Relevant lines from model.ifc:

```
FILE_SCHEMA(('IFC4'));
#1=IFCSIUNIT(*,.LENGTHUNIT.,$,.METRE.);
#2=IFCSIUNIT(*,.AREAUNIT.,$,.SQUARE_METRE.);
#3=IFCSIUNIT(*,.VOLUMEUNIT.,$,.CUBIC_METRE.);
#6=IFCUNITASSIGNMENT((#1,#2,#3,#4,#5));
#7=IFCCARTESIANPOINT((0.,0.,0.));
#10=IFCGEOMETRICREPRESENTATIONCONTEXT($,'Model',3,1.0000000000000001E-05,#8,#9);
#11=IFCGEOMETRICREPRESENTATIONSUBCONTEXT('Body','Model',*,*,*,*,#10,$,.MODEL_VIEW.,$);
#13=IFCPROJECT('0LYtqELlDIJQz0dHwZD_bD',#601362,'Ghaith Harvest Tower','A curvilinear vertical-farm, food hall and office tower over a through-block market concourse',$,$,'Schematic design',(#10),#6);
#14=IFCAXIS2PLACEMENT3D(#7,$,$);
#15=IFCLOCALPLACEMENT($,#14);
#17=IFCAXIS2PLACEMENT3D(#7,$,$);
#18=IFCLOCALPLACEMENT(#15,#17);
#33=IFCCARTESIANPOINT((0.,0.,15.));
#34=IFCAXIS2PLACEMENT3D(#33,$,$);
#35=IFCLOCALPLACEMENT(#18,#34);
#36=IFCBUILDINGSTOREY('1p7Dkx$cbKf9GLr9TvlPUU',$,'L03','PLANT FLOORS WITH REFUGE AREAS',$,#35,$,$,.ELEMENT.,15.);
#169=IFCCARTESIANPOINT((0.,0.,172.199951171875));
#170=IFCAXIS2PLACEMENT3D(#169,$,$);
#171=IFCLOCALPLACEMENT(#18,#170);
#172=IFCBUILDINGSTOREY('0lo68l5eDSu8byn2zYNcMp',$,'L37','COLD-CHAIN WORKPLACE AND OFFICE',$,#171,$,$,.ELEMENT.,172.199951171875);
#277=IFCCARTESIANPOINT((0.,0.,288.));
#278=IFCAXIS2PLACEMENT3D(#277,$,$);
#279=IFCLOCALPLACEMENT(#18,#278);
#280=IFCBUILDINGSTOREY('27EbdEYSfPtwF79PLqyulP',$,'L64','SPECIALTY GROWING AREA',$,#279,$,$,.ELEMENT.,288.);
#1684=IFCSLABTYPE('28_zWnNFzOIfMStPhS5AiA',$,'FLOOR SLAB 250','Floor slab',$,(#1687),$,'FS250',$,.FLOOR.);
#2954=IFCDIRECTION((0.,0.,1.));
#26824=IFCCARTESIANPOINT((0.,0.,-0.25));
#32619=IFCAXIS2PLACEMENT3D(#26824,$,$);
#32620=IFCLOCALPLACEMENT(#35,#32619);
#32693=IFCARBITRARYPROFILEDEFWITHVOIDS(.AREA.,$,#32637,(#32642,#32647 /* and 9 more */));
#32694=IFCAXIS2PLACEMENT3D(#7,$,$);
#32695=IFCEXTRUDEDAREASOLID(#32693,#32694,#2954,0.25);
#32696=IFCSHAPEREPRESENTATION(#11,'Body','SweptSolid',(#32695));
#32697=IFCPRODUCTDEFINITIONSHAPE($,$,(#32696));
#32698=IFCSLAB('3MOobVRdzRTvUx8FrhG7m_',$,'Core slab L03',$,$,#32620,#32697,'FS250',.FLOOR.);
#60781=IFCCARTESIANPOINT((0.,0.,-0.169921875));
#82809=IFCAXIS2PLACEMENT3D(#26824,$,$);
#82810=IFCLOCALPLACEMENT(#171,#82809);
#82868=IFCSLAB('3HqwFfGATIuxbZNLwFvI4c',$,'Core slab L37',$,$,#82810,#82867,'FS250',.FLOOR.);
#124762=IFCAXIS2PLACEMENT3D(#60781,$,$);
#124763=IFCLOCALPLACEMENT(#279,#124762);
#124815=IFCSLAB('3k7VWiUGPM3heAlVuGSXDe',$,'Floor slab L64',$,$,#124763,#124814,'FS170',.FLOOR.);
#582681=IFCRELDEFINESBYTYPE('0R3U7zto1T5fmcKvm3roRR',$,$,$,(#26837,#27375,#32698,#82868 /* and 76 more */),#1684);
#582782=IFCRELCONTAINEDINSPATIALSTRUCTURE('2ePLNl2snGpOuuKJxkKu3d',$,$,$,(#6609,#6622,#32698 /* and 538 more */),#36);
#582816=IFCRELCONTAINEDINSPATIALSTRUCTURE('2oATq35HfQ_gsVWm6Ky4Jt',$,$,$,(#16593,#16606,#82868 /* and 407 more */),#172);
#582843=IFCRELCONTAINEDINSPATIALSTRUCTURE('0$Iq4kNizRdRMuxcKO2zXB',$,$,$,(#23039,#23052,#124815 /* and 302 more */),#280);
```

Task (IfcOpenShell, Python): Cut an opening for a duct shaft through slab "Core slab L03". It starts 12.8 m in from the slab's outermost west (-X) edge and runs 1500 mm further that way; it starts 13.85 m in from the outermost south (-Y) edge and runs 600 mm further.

```python
import numpy as np
import ifcopenshell
import ifcopenshell.api.feature
import ifcopenshell.api.geometry
import ifcopenshell.api.root
import ifcopenshell.geom
import ifcopenshell.util.placement
import ifcopenshell.util.representation
import ifcopenshell.util.shape
import ifcopenshell.util.unit

model = ifcopenshell.open("model.ifc")
unit_scale = ifcopenshell.util.unit.calculate_unit_scale(model)
settings = ifcopenshell.geom.settings()


def volume(element):
    """Net volume in cubic metres, openings subtracted."""
    shape = ifcopenshell.geom.create_shape(settings, element)
    return ifcopenshell.util.shape.get_volume(shape.geometry)


slab = model.by_guid("3MOobVRdzRTvUx8FrhG7m_")
before = volume(slab)

# Extent in the slab's own axes, in metres. The edges named are its -X and -Y sides.
slab_shape = ifcopenshell.geom.create_shape(settings, slab)
vertices = ifcopenshell.util.shape.get_vertices(slab_shape.geometry)
x_min, y_min, bottom = vertices.min(axis=0)
top = vertices[:, 2].max()

opening = ifcopenshell.api.root.create_entity(model, ifc_class="IfcOpeningElement", name="Duct shaft opening", predefined_type="OPENING")
context = ifcopenshell.util.representation.get_context(model, "Model", "Body", "MODEL_VIEW")
width, depth = 1.5, 0.6
outline = [(0.0, 0.0), (width, 0.0), (width, depth), (0.0, depth), (0.0, 0.0)]
# Overshoot both faces by 50 mm so the cut is clean.
shape = ifcopenshell.api.geometry.add_slab_representation(
    model, context=context, depth=top - bottom + 0.1, polyline=outline
)
ifcopenshell.api.geometry.assign_representation(model, product=opening, representation=shape)

matrix = ifcopenshell.util.placement.get_local_placement(slab.ObjectPlacement)
matrix[:, 3] = matrix @ np.append(np.array([x_min + 12.8, y_min + 13.85, bottom - 0.05]) / unit_scale, 1.0)
ifcopenshell.api.geometry.edit_object_placement(model, product=opening, matrix=matrix, is_si=False)
ifcopenshell.api.feature.add_feature(model, feature=opening, element=slab)

after = volume(slab)

print(f"slab volume {before:.3f} -> {after:.3f} m3")

model.write("model-out.ifc")
```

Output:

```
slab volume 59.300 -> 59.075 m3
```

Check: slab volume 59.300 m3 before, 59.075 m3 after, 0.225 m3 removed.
